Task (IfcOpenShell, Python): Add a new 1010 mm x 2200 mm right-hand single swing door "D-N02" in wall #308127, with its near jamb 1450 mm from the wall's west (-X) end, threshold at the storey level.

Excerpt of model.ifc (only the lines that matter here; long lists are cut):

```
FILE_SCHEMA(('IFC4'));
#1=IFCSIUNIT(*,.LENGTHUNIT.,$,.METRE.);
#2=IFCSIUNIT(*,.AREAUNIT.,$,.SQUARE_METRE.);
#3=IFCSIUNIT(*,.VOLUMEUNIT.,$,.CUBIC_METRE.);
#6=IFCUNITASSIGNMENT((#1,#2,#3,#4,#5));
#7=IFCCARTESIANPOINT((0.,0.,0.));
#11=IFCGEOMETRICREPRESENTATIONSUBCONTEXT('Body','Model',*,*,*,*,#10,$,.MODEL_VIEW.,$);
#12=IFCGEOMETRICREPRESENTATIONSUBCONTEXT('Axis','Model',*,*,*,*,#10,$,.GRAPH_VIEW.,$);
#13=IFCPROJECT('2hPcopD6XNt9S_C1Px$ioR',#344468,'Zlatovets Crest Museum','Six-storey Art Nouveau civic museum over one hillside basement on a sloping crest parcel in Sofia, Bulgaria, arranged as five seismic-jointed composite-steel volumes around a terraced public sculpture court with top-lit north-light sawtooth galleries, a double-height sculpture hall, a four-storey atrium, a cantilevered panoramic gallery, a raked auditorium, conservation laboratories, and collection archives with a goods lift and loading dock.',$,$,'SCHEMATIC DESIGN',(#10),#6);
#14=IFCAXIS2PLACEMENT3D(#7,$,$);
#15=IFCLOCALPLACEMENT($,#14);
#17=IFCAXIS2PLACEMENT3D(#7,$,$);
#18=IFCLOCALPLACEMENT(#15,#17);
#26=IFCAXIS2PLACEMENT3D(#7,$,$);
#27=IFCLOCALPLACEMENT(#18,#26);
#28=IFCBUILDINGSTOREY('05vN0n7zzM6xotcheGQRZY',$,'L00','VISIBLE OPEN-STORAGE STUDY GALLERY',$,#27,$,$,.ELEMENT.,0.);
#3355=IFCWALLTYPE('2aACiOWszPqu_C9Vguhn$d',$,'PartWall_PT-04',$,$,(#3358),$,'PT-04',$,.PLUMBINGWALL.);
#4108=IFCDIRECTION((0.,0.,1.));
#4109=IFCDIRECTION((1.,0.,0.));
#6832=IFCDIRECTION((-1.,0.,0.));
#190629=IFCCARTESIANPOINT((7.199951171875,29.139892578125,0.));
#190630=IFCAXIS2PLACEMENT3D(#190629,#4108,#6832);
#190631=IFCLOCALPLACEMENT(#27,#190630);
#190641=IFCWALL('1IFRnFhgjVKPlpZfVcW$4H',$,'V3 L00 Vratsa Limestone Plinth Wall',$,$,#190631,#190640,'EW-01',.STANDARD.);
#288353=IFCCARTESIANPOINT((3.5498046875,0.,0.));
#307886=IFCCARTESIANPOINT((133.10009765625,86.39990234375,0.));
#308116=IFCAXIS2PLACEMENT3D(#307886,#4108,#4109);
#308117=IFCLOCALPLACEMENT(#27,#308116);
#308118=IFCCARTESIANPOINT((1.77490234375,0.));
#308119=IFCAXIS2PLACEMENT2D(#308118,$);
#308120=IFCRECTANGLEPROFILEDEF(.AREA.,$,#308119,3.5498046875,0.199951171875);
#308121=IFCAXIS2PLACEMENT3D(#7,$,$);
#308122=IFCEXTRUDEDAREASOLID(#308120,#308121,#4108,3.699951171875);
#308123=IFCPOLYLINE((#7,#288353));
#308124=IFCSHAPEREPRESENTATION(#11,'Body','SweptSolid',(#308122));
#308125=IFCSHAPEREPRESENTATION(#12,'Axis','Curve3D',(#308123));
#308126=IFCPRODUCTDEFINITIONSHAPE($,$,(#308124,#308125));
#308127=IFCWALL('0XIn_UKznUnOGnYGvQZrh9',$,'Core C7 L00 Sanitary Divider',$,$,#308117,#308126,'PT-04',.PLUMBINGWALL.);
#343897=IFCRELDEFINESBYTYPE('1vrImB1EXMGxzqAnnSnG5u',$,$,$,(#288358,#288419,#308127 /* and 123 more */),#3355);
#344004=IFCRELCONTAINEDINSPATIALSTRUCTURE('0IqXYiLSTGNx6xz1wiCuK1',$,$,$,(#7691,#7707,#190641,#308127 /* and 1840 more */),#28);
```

```python
import numpy as np
import ifcopenshell
import ifcopenshell.api.feature
import ifcopenshell.api.geometry
import ifcopenshell.api.root
import ifcopenshell.api.spatial
import ifcopenshell.geom
import ifcopenshell.util.element
import ifcopenshell.util.placement
import ifcopenshell.util.representation
import ifcopenshell.util.shape
import ifcopenshell.util.unit

model = ifcopenshell.open("model.ifc")
unit_scale = ifcopenshell.util.unit.calculate_unit_scale(model)
settings = ifcopenshell.geom.settings()


def volume(element):
    """Net volume in cubic metres, openings subtracted."""
    shape = ifcopenshell.geom.create_shape(settings, element)
    return ifcopenshell.util.shape.get_volume(shape.geometry)


wall = model.by_id(308127)
storey = ifcopenshell.util.element.get_container(wall, ifc_class="IfcBuildingStorey")
context = ifcopenshell.util.representation.get_context(model, "Model", "Body", "MODEL_VIEW")
before = volume(wall)

width, height, from_end, sill = 1.01, 2.2, 1.45, 0.0  # metres

# The wall runs along its own X axis, and the end named is its -X end.
wall_shape = ifcopenshell.geom.create_shape(settings, wall)
x, y, z = ifcopenshell.util.shape.get_vertices(wall_shape.geometry).T
start = x.min() + from_end
face, thickness = float(y.min()), float(y.max() - y.min())
wall_matrix = ifcopenshell.util.placement.get_local_placement(wall.ObjectPlacement)
level = ifcopenshell.util.placement.get_local_placement(storey.ObjectPlacement)[2, 3]


def in_wall(x, y):
    """Placement at x, y metres in the wall's axes, at sill height."""
    matrix = wall_matrix.copy()
    matrix[:, 3] = wall_matrix @ np.array([x / unit_scale, y / unit_scale, 0.0, 1.0])
    matrix[2, 3] = level + sill / unit_scale
    return matrix


# Opening: a box that overshoots both wall faces by 50 mm.
opening = ifcopenshell.api.root.create_entity(model, ifc_class="IfcOpeningElement", predefined_type="OPENING")
box = ifcopenshell.api.geometry.add_wall_representation(
    model, context=context, length=width, height=height, thickness=thickness + 0.1
)
ifcopenshell.api.geometry.assign_representation(model, product=opening, representation=box)
ifcopenshell.api.geometry.edit_object_placement(model, product=opening, matrix=in_wall(start, face - 0.05), is_si=False)
ifcopenshell.api.feature.add_feature(model, feature=opening, element=wall)

door = ifcopenshell.api.root.create_entity(model, ifc_class="IfcDoor", name="D-N02", predefined_type="DOOR")
door.OverallWidth, door.OverallHeight = width / unit_scale, height / unit_scale
door.OperationType = "SINGLE_SWING_RIGHT"
body = ifcopenshell.api.geometry.add_door_representation(
    model,
    context=context,
    overall_width=door.OverallWidth,
    overall_height=door.OverallHeight,
    operation_type="SINGLE_SWING_RIGHT",
    lining_properties={"LiningDepth": thickness / unit_scale, "ThresholdDepth": thickness / unit_scale},
)
ifcopenshell.api.geometry.assign_representation(model, product=door, representation=body)
ifcopenshell.api.spatial.assign_container(model, products=[door], relating_structure=storey)
ifcopenshell.api.feature.add_filling(model, opening=opening, element=door)

# The lining spans the wall, so the door starts at the wall face.
ifcopenshell.api.geometry.edit_object_placement(model, product=door, matrix=in_wall(start, face), is_si=False)

after = volume(wall)

print(f"wall volume {before:.3f} -> {after:.3f} m3")

model.write("model_edited.ifc")
```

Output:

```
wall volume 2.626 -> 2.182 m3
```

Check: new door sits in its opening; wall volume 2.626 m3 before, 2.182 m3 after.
